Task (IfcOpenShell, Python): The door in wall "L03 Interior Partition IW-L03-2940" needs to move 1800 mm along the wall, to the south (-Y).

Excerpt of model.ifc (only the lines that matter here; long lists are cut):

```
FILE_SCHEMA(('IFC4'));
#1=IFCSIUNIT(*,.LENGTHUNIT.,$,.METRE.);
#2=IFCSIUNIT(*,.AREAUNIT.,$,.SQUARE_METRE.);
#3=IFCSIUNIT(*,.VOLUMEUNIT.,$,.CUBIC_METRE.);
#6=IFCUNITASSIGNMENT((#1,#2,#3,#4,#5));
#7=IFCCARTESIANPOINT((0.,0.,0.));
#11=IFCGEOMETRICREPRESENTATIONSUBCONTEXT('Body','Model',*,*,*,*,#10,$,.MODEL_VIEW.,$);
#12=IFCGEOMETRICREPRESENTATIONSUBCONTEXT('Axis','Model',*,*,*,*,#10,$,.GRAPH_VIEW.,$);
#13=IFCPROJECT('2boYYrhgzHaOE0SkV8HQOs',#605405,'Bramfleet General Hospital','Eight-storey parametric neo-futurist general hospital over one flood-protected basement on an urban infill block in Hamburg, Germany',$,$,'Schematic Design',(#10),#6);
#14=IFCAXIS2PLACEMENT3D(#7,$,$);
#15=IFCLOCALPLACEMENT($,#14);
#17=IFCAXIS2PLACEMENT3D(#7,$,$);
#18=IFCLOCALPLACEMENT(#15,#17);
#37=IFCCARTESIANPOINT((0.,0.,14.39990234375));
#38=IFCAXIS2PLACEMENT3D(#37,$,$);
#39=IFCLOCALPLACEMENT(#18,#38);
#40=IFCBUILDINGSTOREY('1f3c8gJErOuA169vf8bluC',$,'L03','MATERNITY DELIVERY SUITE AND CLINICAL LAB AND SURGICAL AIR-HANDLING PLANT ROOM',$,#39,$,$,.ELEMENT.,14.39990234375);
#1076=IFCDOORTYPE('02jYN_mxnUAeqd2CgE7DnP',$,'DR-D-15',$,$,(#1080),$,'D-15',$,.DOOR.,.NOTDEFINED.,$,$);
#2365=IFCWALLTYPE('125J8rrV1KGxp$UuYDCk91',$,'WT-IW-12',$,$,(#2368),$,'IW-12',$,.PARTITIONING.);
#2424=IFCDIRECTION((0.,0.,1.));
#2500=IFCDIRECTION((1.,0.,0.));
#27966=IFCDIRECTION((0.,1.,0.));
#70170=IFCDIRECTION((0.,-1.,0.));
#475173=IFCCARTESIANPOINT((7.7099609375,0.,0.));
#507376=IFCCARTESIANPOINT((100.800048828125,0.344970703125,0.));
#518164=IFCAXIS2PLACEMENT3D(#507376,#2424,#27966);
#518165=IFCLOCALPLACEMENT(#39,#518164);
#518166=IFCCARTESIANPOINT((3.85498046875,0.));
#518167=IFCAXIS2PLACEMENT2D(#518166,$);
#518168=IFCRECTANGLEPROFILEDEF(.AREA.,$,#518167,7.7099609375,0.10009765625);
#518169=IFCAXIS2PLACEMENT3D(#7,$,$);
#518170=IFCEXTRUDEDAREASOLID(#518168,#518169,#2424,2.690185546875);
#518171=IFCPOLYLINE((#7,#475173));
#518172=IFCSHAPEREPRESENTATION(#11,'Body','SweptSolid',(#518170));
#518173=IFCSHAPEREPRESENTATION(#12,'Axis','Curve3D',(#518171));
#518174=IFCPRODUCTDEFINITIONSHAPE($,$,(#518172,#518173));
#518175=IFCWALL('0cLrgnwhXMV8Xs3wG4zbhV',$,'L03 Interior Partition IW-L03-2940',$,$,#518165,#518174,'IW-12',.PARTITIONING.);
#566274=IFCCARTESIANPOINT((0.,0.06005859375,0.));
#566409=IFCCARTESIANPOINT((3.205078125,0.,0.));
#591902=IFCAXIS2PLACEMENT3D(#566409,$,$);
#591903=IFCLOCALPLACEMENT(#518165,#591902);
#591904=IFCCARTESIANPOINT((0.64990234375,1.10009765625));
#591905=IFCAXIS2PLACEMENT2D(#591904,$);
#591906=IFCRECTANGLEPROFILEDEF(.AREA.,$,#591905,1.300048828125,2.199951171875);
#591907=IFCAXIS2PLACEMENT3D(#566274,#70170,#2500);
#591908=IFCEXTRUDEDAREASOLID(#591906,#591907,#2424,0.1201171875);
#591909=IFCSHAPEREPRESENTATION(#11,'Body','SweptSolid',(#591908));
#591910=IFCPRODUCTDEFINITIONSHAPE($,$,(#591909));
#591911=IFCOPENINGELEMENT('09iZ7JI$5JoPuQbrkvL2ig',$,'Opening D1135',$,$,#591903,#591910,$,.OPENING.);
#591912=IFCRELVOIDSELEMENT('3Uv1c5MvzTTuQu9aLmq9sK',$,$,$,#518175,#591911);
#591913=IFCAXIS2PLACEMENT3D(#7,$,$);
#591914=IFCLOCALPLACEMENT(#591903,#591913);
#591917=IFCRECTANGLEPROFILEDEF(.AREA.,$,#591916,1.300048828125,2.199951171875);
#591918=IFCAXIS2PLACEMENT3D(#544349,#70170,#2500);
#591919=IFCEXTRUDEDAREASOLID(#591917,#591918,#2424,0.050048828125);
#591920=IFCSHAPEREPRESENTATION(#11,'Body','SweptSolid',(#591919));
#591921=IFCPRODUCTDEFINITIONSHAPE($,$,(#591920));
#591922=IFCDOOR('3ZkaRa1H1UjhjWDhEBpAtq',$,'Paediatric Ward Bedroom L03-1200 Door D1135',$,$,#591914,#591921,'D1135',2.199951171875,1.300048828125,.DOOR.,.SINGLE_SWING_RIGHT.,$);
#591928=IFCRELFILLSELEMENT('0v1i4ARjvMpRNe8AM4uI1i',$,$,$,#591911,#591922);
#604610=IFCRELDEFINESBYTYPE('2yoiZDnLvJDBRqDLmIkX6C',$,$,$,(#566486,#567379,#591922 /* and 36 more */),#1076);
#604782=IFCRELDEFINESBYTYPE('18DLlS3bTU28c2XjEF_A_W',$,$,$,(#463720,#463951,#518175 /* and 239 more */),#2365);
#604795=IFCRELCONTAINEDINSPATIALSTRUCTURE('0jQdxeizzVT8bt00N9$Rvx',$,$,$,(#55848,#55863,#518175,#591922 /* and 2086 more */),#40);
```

```python
import ifcopenshell
import ifcopenshell.api.geometry
import ifcopenshell.util.placement
import ifcopenshell.util.unit

model = ifcopenshell.open("model.ifc")
unit_scale = ifcopenshell.util.unit.calculate_unit_scale(model)

door = model.by_guid("3ZkaRa1H1UjhjWDhEBpAtq")
opening = door.FillsVoids[0].RelatingOpeningElement
wall = opening.VoidsElements[0].RelatingBuildingElement

wall_matrix = ifcopenshell.util.placement.get_local_placement(wall.ObjectPlacement)
shift = wall_matrix[:3, 0] * -1.8 / unit_scale
before = ifcopenshell.util.placement.get_local_placement(door.ObjectPlacement)[:3, 3].copy()

# The door is placed relative to its opening, so it follows when the opening moves.
matrix = ifcopenshell.util.placement.get_local_placement(opening.ObjectPlacement)
matrix[:3, 3] += shift
ifcopenshell.api.geometry.edit_object_placement(
    model, product=opening, matrix=matrix, is_si=False, should_transform_children=True
)

after = ifcopenshell.util.placement.get_local_placement(door.ObjectPlacement)[:3, 3]
print("door moved by", (after - before).round(3) + 0.0)

model.write("model_rev.ifc")
```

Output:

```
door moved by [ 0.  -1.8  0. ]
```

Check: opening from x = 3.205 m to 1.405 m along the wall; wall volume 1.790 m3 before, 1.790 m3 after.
